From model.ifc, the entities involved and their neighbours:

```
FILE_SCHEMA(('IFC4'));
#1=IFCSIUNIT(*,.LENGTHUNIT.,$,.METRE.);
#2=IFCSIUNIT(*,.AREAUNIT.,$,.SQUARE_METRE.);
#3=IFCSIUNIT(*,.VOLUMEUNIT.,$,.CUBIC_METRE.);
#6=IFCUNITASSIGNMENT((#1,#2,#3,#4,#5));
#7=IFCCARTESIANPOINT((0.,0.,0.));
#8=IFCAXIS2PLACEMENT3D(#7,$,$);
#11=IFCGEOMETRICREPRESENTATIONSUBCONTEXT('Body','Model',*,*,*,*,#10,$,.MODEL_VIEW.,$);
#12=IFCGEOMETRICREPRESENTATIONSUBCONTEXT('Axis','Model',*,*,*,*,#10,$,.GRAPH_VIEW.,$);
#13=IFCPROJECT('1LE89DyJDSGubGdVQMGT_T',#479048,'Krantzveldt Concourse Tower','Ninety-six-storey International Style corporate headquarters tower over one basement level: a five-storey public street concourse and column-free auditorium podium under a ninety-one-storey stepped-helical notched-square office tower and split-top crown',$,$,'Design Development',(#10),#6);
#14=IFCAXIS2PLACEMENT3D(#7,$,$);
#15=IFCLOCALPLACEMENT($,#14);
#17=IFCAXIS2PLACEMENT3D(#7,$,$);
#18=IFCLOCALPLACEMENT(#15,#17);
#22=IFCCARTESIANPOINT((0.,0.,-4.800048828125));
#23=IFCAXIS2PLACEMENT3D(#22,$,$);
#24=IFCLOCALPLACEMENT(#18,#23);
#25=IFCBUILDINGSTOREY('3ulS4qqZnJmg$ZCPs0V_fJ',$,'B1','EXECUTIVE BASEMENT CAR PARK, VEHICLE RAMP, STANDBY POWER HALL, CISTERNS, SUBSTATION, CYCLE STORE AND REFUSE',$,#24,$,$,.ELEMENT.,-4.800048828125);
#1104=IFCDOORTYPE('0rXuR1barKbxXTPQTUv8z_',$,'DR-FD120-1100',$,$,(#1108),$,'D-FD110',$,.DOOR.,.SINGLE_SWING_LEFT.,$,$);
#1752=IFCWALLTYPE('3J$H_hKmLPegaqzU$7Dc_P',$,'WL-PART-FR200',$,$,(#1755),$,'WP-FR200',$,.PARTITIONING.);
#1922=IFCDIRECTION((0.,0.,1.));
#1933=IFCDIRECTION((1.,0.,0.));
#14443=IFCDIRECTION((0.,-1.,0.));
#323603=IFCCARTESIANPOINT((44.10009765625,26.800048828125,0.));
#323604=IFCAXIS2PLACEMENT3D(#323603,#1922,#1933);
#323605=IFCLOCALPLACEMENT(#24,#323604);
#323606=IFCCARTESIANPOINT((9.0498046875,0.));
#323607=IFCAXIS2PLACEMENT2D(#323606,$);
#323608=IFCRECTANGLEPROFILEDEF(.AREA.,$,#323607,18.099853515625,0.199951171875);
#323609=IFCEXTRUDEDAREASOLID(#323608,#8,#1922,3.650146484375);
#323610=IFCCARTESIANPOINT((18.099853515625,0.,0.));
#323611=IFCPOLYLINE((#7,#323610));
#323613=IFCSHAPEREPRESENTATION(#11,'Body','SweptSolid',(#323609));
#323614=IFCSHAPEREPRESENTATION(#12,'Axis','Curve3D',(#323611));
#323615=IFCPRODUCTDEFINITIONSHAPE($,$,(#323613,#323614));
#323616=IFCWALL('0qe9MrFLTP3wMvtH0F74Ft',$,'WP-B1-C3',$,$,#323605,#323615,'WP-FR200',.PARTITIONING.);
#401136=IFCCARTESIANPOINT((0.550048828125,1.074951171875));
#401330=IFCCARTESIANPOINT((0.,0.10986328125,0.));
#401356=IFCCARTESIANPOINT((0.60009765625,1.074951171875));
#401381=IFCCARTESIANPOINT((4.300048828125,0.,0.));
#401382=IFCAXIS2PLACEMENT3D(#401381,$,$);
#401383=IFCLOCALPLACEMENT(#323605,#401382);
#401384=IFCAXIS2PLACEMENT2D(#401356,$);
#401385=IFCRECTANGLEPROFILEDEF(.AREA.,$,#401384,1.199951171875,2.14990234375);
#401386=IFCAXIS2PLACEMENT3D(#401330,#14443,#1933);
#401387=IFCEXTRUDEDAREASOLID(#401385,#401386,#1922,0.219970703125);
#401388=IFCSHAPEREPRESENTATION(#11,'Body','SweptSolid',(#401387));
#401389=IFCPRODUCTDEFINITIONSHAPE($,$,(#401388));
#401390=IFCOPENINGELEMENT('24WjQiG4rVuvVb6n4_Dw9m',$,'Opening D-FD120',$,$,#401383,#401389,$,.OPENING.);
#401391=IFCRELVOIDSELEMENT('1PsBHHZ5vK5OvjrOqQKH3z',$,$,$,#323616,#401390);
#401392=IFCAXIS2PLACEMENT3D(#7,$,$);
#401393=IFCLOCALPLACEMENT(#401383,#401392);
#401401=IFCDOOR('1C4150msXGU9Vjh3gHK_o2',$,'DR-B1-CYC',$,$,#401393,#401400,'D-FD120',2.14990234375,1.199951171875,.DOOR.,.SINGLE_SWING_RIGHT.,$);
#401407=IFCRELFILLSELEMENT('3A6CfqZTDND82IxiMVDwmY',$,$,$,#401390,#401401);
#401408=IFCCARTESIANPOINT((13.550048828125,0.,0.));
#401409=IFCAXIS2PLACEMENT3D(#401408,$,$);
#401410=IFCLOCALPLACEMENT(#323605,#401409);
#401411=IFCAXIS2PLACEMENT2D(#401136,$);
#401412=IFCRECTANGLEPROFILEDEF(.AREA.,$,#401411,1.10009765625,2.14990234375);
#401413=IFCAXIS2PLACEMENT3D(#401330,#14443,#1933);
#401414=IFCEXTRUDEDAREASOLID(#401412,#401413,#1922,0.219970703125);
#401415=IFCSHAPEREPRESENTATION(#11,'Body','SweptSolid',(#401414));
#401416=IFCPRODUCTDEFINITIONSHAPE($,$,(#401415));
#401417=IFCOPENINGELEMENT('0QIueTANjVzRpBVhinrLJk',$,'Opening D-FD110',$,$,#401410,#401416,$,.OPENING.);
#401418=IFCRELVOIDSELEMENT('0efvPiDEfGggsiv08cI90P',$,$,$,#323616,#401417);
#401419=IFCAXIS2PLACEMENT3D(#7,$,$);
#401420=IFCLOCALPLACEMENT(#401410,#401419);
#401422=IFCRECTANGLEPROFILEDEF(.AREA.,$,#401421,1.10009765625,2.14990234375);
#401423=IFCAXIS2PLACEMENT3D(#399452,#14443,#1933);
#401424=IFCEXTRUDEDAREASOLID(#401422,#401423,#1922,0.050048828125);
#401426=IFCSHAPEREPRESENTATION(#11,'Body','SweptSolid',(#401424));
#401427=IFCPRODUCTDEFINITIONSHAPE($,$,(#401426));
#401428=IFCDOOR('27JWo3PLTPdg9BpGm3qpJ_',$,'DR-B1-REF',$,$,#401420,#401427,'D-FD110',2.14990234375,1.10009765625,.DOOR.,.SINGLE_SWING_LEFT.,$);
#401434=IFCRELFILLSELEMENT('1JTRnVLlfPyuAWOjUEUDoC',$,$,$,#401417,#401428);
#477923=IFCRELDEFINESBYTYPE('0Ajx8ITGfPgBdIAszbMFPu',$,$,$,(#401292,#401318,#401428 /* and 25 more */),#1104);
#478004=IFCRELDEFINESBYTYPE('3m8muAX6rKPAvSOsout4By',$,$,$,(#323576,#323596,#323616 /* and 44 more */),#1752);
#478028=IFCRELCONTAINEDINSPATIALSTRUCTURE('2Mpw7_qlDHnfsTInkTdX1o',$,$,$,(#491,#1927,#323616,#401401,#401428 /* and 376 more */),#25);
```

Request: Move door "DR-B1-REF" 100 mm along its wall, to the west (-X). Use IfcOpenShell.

```python
import ifcopenshell
import ifcopenshell.api.geometry
import ifcopenshell.util.placement

model = ifcopenshell.open("model.ifc")

door = model.by_id(401428)
opening = door.FillsVoids[0].RelatingOpeningElement
wall = opening.VoidsElements[0].RelatingBuildingElement

wall_matrix = ifcopenshell.util.placement.get_local_placement(wall.ObjectPlacement)
shift = wall_matrix[:3, 0] * -0.1
before = ifcopenshell.util.placement.get_local_placement(door.ObjectPlacement)[:3, 3].copy()

# The door is placed relative to its opening, so it follows when the opening moves.
matrix = ifcopenshell.util.placement.get_local_placement(opening.ObjectPlacement)
matrix[:3, 3] += shift
ifcopenshell.api.geometry.edit_object_placement(
    model, product=opening, matrix=matrix, is_si=False, should_transform_children=True
)

after = ifcopenshell.util.placement.get_local_placement(door.ObjectPlacement)[:3, 3]
print("door moved by", (after - before).round(3) + 0.0)

model.write("model-out.ifc")
```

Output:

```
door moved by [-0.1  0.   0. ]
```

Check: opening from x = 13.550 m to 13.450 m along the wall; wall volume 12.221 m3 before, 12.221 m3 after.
